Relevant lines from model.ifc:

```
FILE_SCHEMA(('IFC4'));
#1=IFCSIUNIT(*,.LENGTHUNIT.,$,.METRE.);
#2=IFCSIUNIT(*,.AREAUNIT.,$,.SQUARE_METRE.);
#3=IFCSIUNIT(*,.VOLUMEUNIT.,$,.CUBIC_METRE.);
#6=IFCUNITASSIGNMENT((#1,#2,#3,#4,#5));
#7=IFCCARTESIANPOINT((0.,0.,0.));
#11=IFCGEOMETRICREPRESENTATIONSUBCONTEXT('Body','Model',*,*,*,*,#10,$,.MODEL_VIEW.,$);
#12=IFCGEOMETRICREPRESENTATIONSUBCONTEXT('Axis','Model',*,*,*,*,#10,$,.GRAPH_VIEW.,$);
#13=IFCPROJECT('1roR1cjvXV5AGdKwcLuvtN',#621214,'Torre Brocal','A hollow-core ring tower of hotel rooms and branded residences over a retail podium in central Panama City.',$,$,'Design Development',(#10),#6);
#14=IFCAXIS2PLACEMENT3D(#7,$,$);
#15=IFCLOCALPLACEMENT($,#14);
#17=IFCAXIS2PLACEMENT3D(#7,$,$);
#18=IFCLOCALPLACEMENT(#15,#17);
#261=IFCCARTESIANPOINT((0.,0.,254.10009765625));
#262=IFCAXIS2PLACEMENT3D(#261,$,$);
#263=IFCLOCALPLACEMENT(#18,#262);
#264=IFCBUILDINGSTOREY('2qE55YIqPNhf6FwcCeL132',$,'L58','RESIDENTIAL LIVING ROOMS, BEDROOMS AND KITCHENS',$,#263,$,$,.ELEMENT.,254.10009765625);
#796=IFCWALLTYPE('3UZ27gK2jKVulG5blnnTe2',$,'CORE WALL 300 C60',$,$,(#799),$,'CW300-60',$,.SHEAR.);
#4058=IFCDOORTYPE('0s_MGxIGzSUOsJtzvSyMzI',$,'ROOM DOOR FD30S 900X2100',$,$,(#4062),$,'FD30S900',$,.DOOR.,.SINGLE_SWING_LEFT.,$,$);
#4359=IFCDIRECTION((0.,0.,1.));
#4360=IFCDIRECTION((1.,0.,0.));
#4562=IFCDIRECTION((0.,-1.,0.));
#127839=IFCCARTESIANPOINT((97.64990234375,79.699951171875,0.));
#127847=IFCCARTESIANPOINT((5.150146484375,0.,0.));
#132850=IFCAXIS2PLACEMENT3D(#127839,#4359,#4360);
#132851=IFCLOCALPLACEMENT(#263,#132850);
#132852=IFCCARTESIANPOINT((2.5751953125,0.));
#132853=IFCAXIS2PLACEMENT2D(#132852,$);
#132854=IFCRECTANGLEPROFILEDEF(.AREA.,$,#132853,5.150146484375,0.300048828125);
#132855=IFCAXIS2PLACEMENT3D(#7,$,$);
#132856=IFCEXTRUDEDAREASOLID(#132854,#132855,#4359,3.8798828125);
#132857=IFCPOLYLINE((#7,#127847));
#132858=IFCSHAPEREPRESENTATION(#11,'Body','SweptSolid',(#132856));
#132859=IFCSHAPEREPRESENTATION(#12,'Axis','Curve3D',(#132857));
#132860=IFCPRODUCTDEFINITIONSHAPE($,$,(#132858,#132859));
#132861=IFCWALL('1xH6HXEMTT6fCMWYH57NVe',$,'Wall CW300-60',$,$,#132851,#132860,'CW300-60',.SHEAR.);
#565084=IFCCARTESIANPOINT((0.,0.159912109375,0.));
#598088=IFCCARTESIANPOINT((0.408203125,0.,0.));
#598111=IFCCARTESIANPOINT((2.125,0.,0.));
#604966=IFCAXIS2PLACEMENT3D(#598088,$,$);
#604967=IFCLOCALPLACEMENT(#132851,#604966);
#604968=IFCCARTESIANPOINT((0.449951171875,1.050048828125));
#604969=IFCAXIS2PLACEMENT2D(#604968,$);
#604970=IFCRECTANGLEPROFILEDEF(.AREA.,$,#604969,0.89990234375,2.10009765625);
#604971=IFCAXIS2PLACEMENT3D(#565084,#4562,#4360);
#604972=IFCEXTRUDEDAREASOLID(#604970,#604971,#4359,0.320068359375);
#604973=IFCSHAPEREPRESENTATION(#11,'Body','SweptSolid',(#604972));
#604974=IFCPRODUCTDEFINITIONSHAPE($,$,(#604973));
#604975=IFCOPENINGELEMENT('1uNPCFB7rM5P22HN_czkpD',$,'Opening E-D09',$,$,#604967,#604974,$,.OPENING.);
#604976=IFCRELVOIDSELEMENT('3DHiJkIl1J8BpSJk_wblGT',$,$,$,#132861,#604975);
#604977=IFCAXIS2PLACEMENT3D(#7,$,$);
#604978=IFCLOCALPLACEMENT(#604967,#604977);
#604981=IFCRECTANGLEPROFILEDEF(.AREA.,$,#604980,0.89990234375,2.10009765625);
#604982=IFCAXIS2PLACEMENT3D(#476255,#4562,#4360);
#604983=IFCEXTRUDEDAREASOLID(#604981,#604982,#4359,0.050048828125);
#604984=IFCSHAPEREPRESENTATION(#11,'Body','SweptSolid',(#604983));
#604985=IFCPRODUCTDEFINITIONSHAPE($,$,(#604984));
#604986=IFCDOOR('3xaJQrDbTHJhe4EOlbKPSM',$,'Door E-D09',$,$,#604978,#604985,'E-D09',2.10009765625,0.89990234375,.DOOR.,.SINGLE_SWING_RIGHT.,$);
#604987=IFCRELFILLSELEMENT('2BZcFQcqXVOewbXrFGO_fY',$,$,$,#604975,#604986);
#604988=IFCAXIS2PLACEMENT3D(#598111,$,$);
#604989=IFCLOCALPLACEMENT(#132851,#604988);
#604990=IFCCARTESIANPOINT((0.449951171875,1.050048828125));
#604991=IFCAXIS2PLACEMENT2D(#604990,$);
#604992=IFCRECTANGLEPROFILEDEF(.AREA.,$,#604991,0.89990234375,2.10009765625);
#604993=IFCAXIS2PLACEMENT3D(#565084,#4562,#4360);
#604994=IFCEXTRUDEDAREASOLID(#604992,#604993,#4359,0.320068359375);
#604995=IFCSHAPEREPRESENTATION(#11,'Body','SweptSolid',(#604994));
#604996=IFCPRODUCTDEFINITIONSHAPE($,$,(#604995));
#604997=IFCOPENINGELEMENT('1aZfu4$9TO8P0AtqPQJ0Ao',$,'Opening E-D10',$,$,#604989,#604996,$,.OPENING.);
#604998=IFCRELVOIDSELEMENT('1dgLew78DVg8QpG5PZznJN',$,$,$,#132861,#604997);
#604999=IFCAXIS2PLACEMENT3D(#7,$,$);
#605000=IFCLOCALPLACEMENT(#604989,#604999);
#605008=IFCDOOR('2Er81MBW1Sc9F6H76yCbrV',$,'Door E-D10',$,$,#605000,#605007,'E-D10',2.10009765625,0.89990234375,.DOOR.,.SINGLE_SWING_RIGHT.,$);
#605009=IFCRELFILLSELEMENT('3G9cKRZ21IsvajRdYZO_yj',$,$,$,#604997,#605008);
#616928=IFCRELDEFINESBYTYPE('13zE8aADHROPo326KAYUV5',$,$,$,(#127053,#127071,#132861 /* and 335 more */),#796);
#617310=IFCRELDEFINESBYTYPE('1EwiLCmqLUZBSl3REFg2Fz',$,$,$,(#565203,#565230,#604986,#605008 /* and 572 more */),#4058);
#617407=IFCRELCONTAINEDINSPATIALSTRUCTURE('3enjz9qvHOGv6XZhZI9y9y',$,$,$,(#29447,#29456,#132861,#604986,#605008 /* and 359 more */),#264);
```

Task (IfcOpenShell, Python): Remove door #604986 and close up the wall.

```python
import ifcopenshell
import ifcopenshell.api.feature
import ifcopenshell.api.root
import ifcopenshell.geom
import ifcopenshell.util.shape

model = ifcopenshell.open("model.ifc")
settings = ifcopenshell.geom.settings()


def volume(element):
    """Net volume in cubic metres, openings subtracted."""
    shape = ifcopenshell.geom.create_shape(settings, element)
    return ifcopenshell.util.shape.get_volume(shape.geometry)


door = model.by_guid("3xaJQrDbTHJhe4EOlbKPSM")
opening = door.FillsVoids[0].RelatingOpeningElement
wall = opening.VoidsElements[0].RelatingBuildingElement
before = volume(wall)

ifcopenshell.api.root.remove_product(model, product=door)
ifcopenshell.api.feature.remove_feature(model, feature=opening)

after = volume(wall)

print(f"wall volume {before:.3f} -> {after:.3f} m3")

model.write("model_edited.ifc")
```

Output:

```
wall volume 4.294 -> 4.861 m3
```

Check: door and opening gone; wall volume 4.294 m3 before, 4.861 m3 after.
